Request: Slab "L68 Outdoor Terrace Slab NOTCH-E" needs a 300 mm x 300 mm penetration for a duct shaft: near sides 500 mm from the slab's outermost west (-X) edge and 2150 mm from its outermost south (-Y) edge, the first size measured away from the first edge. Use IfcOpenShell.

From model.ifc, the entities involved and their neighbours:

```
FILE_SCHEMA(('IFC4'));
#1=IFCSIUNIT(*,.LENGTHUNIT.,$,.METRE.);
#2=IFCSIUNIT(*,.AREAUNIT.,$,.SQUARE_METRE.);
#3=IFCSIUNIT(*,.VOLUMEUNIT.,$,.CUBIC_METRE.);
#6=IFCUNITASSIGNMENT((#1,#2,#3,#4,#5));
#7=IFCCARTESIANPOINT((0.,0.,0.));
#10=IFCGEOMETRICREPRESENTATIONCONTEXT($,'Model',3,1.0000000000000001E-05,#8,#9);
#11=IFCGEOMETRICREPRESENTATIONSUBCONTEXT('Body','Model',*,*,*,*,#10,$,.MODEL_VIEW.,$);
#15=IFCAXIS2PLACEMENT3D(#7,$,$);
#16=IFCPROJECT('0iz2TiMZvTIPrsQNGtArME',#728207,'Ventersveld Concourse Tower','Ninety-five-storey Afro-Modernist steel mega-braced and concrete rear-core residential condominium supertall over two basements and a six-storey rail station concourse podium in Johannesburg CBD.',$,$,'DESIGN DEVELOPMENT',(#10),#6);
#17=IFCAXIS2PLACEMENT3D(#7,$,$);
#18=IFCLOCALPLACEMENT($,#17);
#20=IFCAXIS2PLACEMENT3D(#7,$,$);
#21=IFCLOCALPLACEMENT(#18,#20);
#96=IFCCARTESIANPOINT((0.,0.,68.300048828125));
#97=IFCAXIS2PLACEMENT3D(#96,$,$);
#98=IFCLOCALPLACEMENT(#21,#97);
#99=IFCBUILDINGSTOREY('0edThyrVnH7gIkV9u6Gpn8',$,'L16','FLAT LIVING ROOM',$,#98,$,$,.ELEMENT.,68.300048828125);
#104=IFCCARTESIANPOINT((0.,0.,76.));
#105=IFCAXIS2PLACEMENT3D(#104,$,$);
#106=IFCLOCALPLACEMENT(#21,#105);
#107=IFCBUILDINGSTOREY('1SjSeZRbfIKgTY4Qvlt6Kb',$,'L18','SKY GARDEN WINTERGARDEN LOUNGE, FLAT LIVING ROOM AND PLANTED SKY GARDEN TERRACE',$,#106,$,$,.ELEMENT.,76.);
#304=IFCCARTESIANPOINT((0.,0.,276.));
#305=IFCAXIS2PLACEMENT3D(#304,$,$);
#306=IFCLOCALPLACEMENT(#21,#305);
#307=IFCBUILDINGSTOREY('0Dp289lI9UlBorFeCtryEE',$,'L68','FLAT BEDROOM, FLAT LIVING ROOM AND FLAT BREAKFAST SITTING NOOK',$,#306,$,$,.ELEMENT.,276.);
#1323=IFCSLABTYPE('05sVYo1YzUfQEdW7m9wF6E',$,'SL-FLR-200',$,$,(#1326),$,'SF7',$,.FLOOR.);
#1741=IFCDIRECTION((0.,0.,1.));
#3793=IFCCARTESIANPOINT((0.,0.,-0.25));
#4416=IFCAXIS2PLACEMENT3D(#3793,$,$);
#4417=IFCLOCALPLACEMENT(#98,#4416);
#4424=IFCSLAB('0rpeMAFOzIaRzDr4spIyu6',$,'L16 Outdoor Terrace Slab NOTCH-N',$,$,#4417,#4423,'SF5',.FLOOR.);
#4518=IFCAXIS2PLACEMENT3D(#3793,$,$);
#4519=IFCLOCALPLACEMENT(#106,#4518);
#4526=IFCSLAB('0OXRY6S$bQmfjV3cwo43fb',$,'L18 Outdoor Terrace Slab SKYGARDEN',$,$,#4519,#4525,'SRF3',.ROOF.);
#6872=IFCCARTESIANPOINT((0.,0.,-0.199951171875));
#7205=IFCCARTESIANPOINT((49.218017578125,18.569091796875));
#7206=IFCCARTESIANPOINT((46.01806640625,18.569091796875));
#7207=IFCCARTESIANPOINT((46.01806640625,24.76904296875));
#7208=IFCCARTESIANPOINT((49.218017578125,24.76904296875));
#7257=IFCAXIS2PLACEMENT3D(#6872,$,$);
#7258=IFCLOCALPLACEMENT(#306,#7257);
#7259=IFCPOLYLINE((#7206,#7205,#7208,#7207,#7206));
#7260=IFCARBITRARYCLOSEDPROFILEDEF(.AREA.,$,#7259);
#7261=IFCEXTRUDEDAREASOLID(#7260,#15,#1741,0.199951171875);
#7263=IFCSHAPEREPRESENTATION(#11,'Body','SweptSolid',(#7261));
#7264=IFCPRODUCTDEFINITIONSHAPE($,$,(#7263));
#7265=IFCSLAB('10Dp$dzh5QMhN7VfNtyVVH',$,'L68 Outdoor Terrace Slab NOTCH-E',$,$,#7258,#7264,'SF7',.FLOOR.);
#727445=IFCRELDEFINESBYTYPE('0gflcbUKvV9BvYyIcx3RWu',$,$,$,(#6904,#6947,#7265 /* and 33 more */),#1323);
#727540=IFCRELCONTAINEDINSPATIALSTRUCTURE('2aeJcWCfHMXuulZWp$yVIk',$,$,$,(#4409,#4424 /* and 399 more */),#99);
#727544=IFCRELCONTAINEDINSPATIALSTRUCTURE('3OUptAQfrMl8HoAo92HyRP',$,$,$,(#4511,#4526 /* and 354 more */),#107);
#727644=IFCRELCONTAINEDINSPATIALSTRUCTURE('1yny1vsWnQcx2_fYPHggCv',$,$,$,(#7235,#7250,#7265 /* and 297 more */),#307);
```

```python
import numpy as np
import ifcopenshell
import ifcopenshell.api.feature
import ifcopenshell.api.geometry
import ifcopenshell.api.root
import ifcopenshell.geom
import ifcopenshell.util.placement
import ifcopenshell.util.representation
import ifcopenshell.util.shape
import ifcopenshell.util.unit

model = ifcopenshell.open("model.ifc")
unit_scale = ifcopenshell.util.unit.calculate_unit_scale(model)
settings = ifcopenshell.geom.settings()


def volume(element):
    """Net volume in cubic metres, openings subtracted."""
    shape = ifcopenshell.geom.create_shape(settings, element)
    return ifcopenshell.util.shape.get_volume(shape.geometry)


slab = model.by_id(7265)
before = volume(slab)

# Extent in the slab's own axes, in metres. The edges named are its -X and -Y sides.
slab_shape = ifcopenshell.geom.create_shape(settings, slab)
vertices = ifcopenshell.util.shape.get_vertices(slab_shape.geometry)
x_min, y_min, bottom = vertices.min(axis=0)
top = vertices[:, 2].max()

opening = ifcopenshell.api.root.create_entity(model, ifc_class="IfcOpeningElement", name="Duct shaft opening", predefined_type="OPENING")
context = ifcopenshell.util.representation.get_context(model, "Model", "Body", "MODEL_VIEW")
width, depth = 0.3, 0.3
outline = [(0.0, 0.0), (width, 0.0), (width, depth), (0.0, depth), (0.0, 0.0)]
# Overshoot both faces by 50 mm so the cut is clean.
shape = ifcopenshell.api.geometry.add_slab_representation(
    model, context=context, depth=top - bottom + 0.1, polyline=outline
)
ifcopenshell.api.geometry.assign_representation(model, product=opening, representation=shape)

matrix = ifcopenshell.util.placement.get_local_placement(slab.ObjectPlacement)
matrix[:, 3] = matrix @ np.append(np.array([x_min + 0.5, y_min + 2.15, bottom - 0.05]) / unit_scale, 1.0)
ifcopenshell.api.geometry.edit_object_placement(model, product=opening, matrix=matrix, is_si=False)
ifcopenshell.api.feature.add_feature(model, feature=opening, element=slab)

after = volume(slab)

print(f"slab volume {before:.3f} -> {after:.3f} m3")

model.write("model_rev.ifc")
```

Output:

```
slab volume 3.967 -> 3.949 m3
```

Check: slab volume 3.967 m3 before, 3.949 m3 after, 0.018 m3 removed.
